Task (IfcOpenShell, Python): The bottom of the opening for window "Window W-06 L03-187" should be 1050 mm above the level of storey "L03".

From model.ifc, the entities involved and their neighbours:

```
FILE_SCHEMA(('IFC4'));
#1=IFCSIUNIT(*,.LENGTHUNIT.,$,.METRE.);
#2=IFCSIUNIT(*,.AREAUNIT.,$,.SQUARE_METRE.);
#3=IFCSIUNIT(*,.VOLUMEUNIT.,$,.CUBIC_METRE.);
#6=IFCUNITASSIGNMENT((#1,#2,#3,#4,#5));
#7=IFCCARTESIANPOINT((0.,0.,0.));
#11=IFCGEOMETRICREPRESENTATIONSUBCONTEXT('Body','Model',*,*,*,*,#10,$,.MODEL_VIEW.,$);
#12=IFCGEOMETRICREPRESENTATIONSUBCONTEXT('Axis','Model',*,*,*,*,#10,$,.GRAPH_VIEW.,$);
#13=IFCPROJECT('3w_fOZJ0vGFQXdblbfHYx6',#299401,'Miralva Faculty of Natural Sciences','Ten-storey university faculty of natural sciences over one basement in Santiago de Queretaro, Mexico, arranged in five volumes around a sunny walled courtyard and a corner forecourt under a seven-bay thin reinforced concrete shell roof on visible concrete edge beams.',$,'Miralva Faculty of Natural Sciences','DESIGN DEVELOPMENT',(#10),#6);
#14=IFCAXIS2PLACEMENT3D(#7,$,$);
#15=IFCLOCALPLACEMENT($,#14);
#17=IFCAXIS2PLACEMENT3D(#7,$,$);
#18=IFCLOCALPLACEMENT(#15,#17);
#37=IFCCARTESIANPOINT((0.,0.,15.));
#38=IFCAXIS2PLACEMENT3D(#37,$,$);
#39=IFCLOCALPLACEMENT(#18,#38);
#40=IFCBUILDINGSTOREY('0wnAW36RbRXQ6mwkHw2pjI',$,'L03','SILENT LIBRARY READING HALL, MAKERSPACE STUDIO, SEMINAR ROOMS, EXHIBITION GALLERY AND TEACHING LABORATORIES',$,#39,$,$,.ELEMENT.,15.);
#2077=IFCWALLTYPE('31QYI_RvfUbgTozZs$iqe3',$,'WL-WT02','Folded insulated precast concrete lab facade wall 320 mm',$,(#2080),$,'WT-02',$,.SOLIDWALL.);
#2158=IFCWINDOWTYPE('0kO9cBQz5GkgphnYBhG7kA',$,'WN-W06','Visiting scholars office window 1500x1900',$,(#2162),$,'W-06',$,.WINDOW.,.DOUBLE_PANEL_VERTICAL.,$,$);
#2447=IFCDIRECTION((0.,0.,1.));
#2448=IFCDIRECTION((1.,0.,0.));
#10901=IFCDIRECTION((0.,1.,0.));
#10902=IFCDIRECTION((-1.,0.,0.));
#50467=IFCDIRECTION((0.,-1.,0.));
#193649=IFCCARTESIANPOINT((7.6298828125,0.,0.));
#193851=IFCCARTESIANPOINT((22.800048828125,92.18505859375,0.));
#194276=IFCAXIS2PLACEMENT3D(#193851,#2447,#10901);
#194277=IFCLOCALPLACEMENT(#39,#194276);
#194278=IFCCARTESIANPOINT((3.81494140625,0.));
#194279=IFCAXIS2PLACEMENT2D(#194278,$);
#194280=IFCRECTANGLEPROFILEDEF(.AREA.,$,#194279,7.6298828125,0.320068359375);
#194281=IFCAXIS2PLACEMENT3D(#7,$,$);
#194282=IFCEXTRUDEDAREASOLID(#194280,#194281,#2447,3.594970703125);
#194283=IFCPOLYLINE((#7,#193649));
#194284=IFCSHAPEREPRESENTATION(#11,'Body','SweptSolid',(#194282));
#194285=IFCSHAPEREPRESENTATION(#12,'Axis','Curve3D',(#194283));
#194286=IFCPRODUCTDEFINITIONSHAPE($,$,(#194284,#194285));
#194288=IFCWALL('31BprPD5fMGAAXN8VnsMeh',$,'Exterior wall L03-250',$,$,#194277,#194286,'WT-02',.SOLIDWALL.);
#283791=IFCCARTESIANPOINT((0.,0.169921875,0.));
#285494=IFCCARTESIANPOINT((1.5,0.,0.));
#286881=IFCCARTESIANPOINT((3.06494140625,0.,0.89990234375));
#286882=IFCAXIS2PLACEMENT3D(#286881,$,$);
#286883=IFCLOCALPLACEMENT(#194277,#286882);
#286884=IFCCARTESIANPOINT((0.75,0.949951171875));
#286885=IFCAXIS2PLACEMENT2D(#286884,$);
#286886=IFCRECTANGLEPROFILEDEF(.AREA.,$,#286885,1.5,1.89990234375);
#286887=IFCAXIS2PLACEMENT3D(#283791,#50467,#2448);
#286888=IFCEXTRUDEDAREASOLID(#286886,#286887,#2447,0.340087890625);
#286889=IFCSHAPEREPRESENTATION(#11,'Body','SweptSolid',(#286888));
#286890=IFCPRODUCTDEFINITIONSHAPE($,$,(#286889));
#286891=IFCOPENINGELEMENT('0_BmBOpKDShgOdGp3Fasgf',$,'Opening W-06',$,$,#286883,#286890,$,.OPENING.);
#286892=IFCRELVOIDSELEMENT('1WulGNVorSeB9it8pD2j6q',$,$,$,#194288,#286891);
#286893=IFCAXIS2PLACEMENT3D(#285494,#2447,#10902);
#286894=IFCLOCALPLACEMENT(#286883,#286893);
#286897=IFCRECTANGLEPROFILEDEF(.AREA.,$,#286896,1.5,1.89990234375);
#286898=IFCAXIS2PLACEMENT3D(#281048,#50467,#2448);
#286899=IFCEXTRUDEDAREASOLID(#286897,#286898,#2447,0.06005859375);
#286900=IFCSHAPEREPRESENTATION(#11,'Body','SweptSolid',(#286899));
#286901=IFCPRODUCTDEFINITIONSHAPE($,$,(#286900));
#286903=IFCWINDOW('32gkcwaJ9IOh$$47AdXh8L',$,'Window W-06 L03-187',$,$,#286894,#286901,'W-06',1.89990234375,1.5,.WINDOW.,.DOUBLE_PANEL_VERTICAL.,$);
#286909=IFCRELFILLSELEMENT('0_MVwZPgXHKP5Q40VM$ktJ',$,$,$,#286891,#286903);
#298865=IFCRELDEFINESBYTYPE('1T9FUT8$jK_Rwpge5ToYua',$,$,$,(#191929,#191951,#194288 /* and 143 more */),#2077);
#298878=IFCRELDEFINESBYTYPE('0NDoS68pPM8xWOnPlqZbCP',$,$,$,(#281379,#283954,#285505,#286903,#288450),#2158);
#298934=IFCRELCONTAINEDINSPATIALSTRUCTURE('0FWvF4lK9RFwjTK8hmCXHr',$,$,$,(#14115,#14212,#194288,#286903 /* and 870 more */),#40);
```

```python
import numpy as np
import ifcopenshell
import ifcopenshell.api.geometry
import ifcopenshell.geom
import ifcopenshell.util.element
import ifcopenshell.util.placement
import ifcopenshell.util.shape
import ifcopenshell.util.unit

model = ifcopenshell.open("model.ifc")
unit_scale = ifcopenshell.util.unit.calculate_unit_scale(model)

window = model.by_guid("32gkcwaJ9IOh$$47AdXh8L")
opening = window.FillsVoids[0].RelatingOpeningElement
storey = ifcopenshell.util.element.get_container(window, ifc_class="IfcBuildingStorey")
level = ifcopenshell.util.placement.get_local_placement(storey.ObjectPlacement)[2, 3]

# The opening's origin need not be at the sill, so measure its lowest point.
shape = ifcopenshell.geom.create_shape(ifcopenshell.geom.settings(), opening)
bottom = ifcopenshell.util.shape.get_shape_bottom_elevation(shape, shape.geometry) / unit_scale
dz = level + 1.05 - bottom

shift = np.array([0.0, 0.0, dz])
# The window is placed relative to its opening, so it follows when the opening moves.
matrix = ifcopenshell.util.placement.get_local_placement(opening.ObjectPlacement)
matrix[:3, 3] += shift
ifcopenshell.api.geometry.edit_object_placement(
    model, product=opening, matrix=matrix, is_si=False, should_transform_children=True
)

print(f"moved by {dz * unit_scale:+.3f} m")

model.write("model_edited.ifc")
```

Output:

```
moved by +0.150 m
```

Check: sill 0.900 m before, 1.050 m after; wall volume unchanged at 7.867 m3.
